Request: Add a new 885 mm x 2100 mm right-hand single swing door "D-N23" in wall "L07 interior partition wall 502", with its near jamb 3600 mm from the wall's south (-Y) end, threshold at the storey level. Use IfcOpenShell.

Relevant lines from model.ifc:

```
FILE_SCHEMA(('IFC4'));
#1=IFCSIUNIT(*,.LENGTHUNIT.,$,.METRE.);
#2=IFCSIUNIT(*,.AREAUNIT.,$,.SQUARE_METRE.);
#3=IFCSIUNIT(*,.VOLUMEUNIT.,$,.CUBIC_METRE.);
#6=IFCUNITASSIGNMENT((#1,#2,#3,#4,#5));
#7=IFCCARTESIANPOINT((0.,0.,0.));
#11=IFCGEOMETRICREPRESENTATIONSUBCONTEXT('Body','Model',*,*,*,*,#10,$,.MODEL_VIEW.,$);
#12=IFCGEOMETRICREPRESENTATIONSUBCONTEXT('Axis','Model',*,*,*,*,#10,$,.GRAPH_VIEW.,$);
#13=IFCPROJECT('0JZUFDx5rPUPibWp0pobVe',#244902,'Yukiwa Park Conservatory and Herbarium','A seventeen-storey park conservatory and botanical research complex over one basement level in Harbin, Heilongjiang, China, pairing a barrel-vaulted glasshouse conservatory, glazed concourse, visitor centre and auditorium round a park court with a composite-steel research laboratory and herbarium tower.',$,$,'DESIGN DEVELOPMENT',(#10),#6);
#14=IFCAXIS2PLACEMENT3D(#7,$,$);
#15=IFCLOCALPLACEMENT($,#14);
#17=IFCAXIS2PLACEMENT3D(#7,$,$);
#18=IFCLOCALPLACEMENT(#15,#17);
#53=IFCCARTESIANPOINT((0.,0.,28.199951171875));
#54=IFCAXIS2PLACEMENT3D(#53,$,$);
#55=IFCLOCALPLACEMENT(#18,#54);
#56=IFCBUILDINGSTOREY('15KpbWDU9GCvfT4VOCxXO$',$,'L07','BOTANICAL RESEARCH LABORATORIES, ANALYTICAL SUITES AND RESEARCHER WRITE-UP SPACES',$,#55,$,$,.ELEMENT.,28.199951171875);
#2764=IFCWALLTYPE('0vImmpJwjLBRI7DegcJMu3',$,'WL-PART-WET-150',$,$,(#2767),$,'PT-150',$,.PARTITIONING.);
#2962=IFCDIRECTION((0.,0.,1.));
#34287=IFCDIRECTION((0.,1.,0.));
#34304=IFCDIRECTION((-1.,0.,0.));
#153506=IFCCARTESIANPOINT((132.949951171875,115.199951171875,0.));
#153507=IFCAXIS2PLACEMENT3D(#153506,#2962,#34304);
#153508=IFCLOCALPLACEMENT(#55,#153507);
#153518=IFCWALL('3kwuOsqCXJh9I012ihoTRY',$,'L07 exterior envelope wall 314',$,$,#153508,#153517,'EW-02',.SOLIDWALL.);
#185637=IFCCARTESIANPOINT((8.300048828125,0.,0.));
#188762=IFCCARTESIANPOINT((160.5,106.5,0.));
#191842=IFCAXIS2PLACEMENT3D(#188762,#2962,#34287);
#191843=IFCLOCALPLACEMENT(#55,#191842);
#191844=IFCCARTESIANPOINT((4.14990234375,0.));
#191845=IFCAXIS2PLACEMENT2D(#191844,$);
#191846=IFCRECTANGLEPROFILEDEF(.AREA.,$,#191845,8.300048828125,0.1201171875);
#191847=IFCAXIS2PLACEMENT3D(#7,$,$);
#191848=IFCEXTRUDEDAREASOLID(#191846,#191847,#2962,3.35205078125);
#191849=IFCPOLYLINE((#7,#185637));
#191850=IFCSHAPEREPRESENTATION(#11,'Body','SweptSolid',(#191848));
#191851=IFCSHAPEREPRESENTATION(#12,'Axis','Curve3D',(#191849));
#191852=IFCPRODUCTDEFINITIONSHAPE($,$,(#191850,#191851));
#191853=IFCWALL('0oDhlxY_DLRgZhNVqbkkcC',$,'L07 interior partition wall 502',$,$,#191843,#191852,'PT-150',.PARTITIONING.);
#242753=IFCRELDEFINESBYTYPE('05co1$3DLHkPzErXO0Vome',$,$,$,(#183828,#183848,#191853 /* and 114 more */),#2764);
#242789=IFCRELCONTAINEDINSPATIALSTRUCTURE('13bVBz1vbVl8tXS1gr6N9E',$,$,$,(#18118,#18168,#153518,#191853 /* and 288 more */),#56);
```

```python
import numpy as np
import ifcopenshell
import ifcopenshell.api.feature
import ifcopenshell.api.geometry
import ifcopenshell.api.root
import ifcopenshell.api.spatial
import ifcopenshell.geom
import ifcopenshell.util.element
import ifcopenshell.util.placement
import ifcopenshell.util.representation
import ifcopenshell.util.shape
import ifcopenshell.util.unit

model = ifcopenshell.open("model.ifc")
unit_scale = ifcopenshell.util.unit.calculate_unit_scale(model)
settings = ifcopenshell.geom.settings()


def volume(element):
    """Net volume in cubic metres, openings subtracted."""
    shape = ifcopenshell.geom.create_shape(settings, element)
    return ifcopenshell.util.shape.get_volume(shape.geometry)


wall = model.by_guid("0oDhlxY_DLRgZhNVqbkkcC")
storey = ifcopenshell.util.element.get_container(wall, ifc_class="IfcBuildingStorey")
context = ifcopenshell.util.representation.get_context(model, "Model", "Body", "MODEL_VIEW")
before = volume(wall)

width, height, from_end, sill = 0.885, 2.1, 3.6, 0.0  # metres

# The wall runs along its own X axis, and the end named is its -X end.
wall_shape = ifcopenshell.geom.create_shape(settings, wall)
x, y, z = ifcopenshell.util.shape.get_vertices(wall_shape.geometry).T
start = x.min() + from_end
face, thickness = float(y.min()), float(y.max() - y.min())
wall_matrix = ifcopenshell.util.placement.get_local_placement(wall.ObjectPlacement)
level = ifcopenshell.util.placement.get_local_placement(storey.ObjectPlacement)[2, 3]


def in_wall(x, y):
    """Placement at x, y metres in the wall's axes, at sill height."""
    matrix = wall_matrix.copy()
    matrix[:, 3] = wall_matrix @ np.array([x / unit_scale, y / unit_scale, 0.0, 1.0])
    matrix[2, 3] = level + sill / unit_scale
    return matrix


# Opening: a box that overshoots both wall faces by 50 mm.
opening = ifcopenshell.api.root.create_entity(model, ifc_class="IfcOpeningElement", predefined_type="OPENING")
box = ifcopenshell.api.geometry.add_wall_representation(
    model, context=context, length=width, height=height, thickness=thickness + 0.1
)
ifcopenshell.api.geometry.assign_representation(model, product=opening, representation=box)
ifcopenshell.api.geometry.edit_object_placement(model, product=opening, matrix=in_wall(start, face - 0.05), is_si=False)
ifcopenshell.api.feature.add_feature(model, feature=opening, element=wall)

door = ifcopenshell.api.root.create_entity(model, ifc_class="IfcDoor", name="D-N23", predefined_type="DOOR")
door.OverallWidth, door.OverallHeight = width / unit_scale, height / unit_scale
door.OperationType = "SINGLE_SWING_RIGHT"
body = ifcopenshell.api.geometry.add_door_representation(
    model,
    context=context,
    overall_width=door.OverallWidth,
    overall_height=door.OverallHeight,
    operation_type="SINGLE_SWING_RIGHT",
    lining_properties={"LiningDepth": thickness / unit_scale, "ThresholdDepth": thickness / unit_scale},
)
ifcopenshell.api.geometry.assign_representation(model, product=door, representation=body)
ifcopenshell.api.spatial.assign_container(model, products=[door], relating_structure=storey)
ifcopenshell.api.feature.add_filling(model, opening=opening, element=door)

# The lining spans the wall, so the door starts at the wall face.
ifcopenshell.api.geometry.edit_object_placement(model, product=door, matrix=in_wall(start, face), is_si=False)

after = volume(wall)

print(f"wall volume {before:.3f} -> {after:.3f} m3")

model.write("model_updated.ifc")
```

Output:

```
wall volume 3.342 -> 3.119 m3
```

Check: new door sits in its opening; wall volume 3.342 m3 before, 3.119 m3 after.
